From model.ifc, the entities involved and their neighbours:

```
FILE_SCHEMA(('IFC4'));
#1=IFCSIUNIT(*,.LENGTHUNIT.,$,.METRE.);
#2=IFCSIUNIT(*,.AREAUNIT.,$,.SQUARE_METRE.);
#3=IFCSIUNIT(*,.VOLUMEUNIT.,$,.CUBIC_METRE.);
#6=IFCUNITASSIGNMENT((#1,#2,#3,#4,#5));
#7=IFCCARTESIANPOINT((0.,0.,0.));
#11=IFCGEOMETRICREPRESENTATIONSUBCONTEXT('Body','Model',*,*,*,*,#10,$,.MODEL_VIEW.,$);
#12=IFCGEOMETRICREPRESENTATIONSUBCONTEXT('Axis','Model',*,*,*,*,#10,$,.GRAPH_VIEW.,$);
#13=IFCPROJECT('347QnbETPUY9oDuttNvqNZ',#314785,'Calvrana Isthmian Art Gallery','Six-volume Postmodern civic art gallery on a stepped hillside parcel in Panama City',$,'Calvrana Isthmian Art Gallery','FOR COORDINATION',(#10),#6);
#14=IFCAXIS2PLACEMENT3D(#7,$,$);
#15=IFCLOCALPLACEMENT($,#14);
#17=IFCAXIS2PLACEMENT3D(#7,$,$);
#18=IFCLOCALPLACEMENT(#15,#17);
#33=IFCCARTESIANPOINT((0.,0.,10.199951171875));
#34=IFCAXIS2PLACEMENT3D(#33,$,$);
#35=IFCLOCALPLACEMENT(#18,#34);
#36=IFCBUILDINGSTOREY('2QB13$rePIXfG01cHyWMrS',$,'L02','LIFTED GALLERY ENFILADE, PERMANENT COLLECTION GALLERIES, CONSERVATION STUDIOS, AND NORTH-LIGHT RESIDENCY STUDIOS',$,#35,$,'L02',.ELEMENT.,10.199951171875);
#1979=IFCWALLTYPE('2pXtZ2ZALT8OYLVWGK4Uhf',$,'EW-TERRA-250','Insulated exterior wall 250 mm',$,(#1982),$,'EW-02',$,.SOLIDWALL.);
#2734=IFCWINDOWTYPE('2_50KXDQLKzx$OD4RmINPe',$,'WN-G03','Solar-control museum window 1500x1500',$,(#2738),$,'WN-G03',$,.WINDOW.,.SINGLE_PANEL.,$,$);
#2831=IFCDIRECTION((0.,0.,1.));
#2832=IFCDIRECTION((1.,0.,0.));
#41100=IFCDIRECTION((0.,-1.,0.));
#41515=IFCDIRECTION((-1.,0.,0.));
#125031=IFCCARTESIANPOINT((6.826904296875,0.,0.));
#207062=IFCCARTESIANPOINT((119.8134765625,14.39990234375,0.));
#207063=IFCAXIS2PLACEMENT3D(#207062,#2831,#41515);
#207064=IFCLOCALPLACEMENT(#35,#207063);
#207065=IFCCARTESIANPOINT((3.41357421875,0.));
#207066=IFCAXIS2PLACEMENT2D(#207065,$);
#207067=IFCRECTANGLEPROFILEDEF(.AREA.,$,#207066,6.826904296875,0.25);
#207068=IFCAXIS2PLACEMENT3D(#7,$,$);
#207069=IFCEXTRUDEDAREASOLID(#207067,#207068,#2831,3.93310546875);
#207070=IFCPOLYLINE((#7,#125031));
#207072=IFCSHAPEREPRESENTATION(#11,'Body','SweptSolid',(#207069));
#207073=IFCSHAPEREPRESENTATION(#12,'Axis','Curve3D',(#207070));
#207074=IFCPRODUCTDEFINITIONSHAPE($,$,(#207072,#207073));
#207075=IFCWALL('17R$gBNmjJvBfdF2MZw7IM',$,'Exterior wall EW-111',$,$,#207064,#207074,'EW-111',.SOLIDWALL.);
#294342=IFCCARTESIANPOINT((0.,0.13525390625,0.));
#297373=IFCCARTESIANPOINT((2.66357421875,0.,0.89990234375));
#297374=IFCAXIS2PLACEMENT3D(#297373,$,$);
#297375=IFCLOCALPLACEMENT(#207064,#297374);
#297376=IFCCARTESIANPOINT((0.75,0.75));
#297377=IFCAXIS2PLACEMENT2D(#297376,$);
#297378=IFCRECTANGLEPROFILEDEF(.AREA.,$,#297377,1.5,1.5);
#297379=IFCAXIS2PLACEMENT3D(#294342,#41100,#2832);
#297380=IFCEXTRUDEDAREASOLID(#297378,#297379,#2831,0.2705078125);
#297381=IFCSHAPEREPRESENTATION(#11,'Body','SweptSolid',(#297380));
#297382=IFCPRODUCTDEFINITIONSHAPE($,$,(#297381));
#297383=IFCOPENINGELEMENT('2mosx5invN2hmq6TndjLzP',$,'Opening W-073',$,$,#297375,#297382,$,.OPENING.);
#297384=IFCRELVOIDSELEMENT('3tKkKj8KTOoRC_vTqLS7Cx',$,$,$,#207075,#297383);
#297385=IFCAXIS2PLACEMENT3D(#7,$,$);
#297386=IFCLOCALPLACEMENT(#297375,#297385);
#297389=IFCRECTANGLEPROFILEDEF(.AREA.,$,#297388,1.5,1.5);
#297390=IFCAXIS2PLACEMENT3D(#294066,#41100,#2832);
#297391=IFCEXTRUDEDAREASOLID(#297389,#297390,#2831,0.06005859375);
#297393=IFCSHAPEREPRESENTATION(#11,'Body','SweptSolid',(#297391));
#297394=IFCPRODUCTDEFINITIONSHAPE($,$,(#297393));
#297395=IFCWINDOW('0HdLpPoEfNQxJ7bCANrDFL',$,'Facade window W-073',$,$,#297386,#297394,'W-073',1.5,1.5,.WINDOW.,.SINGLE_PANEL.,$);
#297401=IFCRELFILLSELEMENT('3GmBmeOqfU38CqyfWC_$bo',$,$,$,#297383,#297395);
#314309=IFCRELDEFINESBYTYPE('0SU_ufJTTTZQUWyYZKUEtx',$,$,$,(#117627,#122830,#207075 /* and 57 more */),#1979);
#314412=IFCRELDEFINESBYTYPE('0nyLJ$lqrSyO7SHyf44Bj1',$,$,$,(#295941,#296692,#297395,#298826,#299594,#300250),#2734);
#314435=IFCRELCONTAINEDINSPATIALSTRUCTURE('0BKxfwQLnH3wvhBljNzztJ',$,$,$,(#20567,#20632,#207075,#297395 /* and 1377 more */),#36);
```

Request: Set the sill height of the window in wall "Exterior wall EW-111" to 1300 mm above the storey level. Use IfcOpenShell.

```python
import numpy as np
import ifcopenshell
import ifcopenshell.api.geometry
import ifcopenshell.geom
import ifcopenshell.util.element
import ifcopenshell.util.placement
import ifcopenshell.util.shape
import ifcopenshell.util.unit

model = ifcopenshell.open("model.ifc")
unit_scale = ifcopenshell.util.unit.calculate_unit_scale(model)

window = model.by_guid("0HdLpPoEfNQxJ7bCANrDFL")
opening = window.FillsVoids[0].RelatingOpeningElement
storey = ifcopenshell.util.element.get_container(window, ifc_class="IfcBuildingStorey")
level = ifcopenshell.util.placement.get_local_placement(storey.ObjectPlacement)[2, 3]

# The opening's origin need not be at the sill, so measure its lowest point.
shape = ifcopenshell.geom.create_shape(ifcopenshell.geom.settings(), opening)
bottom = ifcopenshell.util.shape.get_shape_bottom_elevation(shape, shape.geometry) / unit_scale
dz = level + 1.3 / unit_scale - bottom

shift = np.array([0.0, 0.0, dz])
# The window is placed relative to its opening, so it follows when the opening moves.
matrix = ifcopenshell.util.placement.get_local_placement(opening.ObjectPlacement)
matrix[:3, 3] += shift
ifcopenshell.api.geometry.edit_object_placement(
    model, product=opening, matrix=matrix, is_si=False, should_transform_children=True
)

print(f"moved by {dz * unit_scale:+.3f} m")

model.write("model_v2.ifc")
```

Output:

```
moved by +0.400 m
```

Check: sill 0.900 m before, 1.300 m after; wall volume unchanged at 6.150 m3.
